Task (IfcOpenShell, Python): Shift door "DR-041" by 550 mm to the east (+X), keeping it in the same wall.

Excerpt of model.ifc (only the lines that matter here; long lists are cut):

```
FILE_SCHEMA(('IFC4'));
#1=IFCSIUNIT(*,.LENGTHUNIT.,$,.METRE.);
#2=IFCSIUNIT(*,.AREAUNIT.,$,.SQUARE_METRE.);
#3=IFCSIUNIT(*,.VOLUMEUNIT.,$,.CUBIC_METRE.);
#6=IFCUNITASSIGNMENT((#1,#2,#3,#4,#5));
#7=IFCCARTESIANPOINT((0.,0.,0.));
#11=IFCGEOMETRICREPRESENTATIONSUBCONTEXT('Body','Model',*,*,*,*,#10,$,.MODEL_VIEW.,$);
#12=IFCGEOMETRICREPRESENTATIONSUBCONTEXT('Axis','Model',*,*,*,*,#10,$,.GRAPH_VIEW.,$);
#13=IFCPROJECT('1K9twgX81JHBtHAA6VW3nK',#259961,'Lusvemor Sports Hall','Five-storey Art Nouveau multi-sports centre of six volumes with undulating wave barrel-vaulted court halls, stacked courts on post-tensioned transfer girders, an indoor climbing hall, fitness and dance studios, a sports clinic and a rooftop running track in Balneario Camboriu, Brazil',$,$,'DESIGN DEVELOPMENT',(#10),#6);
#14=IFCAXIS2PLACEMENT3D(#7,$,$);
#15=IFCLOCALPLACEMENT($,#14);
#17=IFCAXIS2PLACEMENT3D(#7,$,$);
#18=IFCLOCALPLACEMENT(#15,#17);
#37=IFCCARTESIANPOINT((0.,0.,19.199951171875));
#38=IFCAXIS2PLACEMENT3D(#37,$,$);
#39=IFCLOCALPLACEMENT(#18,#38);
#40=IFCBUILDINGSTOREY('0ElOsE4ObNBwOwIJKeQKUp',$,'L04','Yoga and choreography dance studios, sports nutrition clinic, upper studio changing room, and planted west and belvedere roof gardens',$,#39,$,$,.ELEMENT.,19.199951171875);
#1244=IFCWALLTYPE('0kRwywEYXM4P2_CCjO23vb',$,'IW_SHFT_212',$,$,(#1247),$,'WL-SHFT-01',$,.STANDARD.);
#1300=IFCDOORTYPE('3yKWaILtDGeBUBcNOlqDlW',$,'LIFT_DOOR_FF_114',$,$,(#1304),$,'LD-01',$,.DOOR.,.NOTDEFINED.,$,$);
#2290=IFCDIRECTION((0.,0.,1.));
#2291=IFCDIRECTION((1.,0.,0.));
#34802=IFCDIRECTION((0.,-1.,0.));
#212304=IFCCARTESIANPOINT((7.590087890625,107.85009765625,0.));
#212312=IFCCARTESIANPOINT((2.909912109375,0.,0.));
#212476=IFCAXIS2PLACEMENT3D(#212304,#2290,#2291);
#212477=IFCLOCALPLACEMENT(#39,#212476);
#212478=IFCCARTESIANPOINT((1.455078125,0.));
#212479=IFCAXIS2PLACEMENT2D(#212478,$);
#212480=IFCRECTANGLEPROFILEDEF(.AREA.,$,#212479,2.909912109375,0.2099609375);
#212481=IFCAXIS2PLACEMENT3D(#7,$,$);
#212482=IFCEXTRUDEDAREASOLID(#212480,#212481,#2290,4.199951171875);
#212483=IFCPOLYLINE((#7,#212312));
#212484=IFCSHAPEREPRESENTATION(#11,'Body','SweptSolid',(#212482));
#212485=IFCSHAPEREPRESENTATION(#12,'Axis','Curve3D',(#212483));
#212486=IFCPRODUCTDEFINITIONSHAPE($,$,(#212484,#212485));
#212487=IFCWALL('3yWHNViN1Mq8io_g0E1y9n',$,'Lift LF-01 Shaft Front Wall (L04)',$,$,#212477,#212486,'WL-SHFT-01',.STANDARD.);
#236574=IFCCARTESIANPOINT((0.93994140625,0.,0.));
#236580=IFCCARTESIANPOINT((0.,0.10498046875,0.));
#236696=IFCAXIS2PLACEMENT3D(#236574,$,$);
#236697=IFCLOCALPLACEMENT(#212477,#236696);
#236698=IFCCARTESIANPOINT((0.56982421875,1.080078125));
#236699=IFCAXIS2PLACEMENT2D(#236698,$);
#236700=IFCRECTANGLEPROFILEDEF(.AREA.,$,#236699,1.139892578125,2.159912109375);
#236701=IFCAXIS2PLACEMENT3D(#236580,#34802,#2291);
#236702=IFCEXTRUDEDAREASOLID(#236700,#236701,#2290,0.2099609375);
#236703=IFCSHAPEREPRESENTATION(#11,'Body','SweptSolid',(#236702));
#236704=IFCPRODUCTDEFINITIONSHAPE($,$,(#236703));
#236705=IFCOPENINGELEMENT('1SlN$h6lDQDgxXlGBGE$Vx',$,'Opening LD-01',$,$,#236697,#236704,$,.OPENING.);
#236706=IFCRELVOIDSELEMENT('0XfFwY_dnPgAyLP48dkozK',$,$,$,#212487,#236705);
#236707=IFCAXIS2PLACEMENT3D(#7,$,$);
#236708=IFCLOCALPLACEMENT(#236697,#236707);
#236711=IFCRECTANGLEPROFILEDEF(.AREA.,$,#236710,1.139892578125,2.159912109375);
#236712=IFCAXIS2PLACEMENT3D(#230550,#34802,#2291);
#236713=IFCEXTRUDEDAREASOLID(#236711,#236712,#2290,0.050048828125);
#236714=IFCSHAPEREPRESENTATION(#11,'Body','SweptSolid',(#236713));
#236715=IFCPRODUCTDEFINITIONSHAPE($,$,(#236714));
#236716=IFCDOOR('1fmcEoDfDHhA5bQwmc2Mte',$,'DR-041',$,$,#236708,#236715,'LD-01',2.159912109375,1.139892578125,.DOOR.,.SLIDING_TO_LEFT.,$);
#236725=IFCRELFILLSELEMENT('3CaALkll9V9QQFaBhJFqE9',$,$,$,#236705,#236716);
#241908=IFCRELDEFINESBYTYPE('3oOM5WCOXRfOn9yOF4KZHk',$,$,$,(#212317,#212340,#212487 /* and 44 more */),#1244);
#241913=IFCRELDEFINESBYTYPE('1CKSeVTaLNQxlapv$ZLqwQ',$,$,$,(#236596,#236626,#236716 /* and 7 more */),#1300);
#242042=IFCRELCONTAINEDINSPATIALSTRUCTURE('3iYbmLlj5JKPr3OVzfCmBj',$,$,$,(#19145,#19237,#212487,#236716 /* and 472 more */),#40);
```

```python
import ifcopenshell
import ifcopenshell.api.geometry
import ifcopenshell.util.placement
import ifcopenshell.util.unit

model = ifcopenshell.open("model.ifc")
unit_scale = ifcopenshell.util.unit.calculate_unit_scale(model)

door = model.by_id(236716)
opening = door.FillsVoids[0].RelatingOpeningElement
wall = opening.VoidsElements[0].RelatingBuildingElement

wall_matrix = ifcopenshell.util.placement.get_local_placement(wall.ObjectPlacement)
shift = wall_matrix[:3, 0] * 0.55 / unit_scale
before = ifcopenshell.util.placement.get_local_placement(door.ObjectPlacement)[:3, 3].copy()

# The door is placed relative to its opening, so it follows when the opening moves.
matrix = ifcopenshell.util.placement.get_local_placement(opening.ObjectPlacement)
matrix[:3, 3] += shift
ifcopenshell.api.geometry.edit_object_placement(
    model, product=opening, matrix=matrix, is_si=False, should_transform_children=True
)

after = ifcopenshell.util.placement.get_local_placement(door.ObjectPlacement)[:3, 3]
print("door moved by", (after - before).round(3) + 0.0)

model.write("model_updated.ifc")
```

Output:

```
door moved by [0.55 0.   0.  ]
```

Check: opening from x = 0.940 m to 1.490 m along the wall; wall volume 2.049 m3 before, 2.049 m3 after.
